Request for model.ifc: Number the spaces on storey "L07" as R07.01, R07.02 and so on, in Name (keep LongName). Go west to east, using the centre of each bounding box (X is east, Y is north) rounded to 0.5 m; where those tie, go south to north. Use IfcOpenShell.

First a look at what the model holds.

```python
import ifcopenshell
import ifcopenshell.util.element
import ifcopenshell.util.placement

model = ifcopenshell.open("model.ifc")
print(model.schema)
storey = next(s for s in model.by_type("IfcBuildingStorey") if s.Name == "L07")
spaces = [e for e in ifcopenshell.util.element.get_decomposition(storey) if e.is_a("IfcSpace")]
for e in sorted(spaces, key=lambda e: e.id()):
    origin = ifcopenshell.util.placement.get_local_placement(e.ObjectPlacement)[:3, 3]
    print(e.id(), e.Name, e.LongName, origin.round(2) + 0.0, sep=" | ")
```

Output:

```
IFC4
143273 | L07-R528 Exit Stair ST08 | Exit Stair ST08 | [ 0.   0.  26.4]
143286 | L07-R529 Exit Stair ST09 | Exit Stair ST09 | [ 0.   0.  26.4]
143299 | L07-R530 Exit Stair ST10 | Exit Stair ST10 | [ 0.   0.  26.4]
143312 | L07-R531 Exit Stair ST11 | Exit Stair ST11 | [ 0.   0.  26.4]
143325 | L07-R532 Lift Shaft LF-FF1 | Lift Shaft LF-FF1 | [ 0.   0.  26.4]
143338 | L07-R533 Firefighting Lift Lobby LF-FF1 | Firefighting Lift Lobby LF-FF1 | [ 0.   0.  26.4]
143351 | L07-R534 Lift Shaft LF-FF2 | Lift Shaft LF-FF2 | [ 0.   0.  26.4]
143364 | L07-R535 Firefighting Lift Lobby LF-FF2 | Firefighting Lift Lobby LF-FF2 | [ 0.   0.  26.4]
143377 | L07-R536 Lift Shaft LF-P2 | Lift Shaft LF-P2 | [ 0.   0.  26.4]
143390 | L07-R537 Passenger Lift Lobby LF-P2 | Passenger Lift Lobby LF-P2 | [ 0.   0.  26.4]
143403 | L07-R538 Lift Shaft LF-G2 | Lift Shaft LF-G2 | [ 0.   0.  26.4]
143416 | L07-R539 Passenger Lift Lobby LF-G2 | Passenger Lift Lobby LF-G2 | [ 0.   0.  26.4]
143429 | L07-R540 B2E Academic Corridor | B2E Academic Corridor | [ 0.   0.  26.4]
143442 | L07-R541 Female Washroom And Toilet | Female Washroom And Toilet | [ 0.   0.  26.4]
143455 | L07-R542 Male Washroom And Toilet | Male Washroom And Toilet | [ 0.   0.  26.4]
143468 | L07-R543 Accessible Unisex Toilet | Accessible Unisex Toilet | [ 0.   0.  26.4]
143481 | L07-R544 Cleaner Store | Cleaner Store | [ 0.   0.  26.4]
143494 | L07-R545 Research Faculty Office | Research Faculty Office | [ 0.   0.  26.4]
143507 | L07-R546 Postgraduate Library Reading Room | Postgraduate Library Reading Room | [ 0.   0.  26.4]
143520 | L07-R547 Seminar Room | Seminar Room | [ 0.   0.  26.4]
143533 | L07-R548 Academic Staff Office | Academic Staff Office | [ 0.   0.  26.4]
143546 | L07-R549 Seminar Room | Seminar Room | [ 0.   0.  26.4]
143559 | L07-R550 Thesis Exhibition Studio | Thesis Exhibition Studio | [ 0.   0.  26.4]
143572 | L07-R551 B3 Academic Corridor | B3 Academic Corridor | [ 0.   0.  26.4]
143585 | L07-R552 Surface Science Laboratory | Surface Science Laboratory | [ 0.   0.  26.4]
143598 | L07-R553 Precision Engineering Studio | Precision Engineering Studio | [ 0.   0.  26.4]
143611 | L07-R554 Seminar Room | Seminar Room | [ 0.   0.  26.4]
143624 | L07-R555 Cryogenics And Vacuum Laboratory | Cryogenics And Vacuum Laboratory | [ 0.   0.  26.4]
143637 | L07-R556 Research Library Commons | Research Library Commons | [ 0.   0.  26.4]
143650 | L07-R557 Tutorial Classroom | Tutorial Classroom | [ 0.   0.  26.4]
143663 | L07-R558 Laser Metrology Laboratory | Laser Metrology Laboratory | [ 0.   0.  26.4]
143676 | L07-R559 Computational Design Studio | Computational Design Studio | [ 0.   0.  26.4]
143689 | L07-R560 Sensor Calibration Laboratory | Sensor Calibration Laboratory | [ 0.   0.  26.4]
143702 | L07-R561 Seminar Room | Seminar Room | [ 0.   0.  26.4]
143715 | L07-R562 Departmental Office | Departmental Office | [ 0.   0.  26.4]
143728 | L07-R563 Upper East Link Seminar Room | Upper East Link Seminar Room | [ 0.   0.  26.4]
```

```python
import ifcopenshell
import ifcopenshell.geom
import ifcopenshell.util.element
import ifcopenshell.util.shape

model = ifcopenshell.open("model.ifc")
settings = ifcopenshell.geom.settings()
settings.set("use-world-coords", True)


def centre(element):
    shape = ifcopenshell.geom.create_shape(settings, element)
    return ifcopenshell.util.shape.get_bbox_centroid(shape.geometry)


storey = next(s for s in model.by_type("IfcBuildingStorey") if s.Name == "L07")
spaces = [e for e in ifcopenshell.util.element.get_decomposition(storey) if e.is_a("IfcSpace")]

# Insertion points can sit at a corner or the storey origin, so sort by the geometry (in metres).
centres = {e: centre(e) for e in spaces}
spaces.sort(key=lambda e: (round(centres[e][0] / 0.5), centres[e][1]))

for i, e in enumerate(spaces, start=1):
    number = f"R07.{i:02d}"
    e.Name = number
    print(e.id(), number)

model.write("model_edited.ifc")
```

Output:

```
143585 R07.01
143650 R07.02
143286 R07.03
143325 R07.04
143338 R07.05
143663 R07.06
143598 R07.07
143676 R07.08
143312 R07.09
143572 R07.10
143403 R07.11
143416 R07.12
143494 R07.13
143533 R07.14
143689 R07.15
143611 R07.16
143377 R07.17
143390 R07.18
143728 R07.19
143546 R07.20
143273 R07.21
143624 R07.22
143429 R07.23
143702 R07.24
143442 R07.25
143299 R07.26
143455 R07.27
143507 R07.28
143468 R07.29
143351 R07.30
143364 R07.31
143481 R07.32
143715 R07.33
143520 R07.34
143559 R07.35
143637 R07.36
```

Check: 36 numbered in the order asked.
